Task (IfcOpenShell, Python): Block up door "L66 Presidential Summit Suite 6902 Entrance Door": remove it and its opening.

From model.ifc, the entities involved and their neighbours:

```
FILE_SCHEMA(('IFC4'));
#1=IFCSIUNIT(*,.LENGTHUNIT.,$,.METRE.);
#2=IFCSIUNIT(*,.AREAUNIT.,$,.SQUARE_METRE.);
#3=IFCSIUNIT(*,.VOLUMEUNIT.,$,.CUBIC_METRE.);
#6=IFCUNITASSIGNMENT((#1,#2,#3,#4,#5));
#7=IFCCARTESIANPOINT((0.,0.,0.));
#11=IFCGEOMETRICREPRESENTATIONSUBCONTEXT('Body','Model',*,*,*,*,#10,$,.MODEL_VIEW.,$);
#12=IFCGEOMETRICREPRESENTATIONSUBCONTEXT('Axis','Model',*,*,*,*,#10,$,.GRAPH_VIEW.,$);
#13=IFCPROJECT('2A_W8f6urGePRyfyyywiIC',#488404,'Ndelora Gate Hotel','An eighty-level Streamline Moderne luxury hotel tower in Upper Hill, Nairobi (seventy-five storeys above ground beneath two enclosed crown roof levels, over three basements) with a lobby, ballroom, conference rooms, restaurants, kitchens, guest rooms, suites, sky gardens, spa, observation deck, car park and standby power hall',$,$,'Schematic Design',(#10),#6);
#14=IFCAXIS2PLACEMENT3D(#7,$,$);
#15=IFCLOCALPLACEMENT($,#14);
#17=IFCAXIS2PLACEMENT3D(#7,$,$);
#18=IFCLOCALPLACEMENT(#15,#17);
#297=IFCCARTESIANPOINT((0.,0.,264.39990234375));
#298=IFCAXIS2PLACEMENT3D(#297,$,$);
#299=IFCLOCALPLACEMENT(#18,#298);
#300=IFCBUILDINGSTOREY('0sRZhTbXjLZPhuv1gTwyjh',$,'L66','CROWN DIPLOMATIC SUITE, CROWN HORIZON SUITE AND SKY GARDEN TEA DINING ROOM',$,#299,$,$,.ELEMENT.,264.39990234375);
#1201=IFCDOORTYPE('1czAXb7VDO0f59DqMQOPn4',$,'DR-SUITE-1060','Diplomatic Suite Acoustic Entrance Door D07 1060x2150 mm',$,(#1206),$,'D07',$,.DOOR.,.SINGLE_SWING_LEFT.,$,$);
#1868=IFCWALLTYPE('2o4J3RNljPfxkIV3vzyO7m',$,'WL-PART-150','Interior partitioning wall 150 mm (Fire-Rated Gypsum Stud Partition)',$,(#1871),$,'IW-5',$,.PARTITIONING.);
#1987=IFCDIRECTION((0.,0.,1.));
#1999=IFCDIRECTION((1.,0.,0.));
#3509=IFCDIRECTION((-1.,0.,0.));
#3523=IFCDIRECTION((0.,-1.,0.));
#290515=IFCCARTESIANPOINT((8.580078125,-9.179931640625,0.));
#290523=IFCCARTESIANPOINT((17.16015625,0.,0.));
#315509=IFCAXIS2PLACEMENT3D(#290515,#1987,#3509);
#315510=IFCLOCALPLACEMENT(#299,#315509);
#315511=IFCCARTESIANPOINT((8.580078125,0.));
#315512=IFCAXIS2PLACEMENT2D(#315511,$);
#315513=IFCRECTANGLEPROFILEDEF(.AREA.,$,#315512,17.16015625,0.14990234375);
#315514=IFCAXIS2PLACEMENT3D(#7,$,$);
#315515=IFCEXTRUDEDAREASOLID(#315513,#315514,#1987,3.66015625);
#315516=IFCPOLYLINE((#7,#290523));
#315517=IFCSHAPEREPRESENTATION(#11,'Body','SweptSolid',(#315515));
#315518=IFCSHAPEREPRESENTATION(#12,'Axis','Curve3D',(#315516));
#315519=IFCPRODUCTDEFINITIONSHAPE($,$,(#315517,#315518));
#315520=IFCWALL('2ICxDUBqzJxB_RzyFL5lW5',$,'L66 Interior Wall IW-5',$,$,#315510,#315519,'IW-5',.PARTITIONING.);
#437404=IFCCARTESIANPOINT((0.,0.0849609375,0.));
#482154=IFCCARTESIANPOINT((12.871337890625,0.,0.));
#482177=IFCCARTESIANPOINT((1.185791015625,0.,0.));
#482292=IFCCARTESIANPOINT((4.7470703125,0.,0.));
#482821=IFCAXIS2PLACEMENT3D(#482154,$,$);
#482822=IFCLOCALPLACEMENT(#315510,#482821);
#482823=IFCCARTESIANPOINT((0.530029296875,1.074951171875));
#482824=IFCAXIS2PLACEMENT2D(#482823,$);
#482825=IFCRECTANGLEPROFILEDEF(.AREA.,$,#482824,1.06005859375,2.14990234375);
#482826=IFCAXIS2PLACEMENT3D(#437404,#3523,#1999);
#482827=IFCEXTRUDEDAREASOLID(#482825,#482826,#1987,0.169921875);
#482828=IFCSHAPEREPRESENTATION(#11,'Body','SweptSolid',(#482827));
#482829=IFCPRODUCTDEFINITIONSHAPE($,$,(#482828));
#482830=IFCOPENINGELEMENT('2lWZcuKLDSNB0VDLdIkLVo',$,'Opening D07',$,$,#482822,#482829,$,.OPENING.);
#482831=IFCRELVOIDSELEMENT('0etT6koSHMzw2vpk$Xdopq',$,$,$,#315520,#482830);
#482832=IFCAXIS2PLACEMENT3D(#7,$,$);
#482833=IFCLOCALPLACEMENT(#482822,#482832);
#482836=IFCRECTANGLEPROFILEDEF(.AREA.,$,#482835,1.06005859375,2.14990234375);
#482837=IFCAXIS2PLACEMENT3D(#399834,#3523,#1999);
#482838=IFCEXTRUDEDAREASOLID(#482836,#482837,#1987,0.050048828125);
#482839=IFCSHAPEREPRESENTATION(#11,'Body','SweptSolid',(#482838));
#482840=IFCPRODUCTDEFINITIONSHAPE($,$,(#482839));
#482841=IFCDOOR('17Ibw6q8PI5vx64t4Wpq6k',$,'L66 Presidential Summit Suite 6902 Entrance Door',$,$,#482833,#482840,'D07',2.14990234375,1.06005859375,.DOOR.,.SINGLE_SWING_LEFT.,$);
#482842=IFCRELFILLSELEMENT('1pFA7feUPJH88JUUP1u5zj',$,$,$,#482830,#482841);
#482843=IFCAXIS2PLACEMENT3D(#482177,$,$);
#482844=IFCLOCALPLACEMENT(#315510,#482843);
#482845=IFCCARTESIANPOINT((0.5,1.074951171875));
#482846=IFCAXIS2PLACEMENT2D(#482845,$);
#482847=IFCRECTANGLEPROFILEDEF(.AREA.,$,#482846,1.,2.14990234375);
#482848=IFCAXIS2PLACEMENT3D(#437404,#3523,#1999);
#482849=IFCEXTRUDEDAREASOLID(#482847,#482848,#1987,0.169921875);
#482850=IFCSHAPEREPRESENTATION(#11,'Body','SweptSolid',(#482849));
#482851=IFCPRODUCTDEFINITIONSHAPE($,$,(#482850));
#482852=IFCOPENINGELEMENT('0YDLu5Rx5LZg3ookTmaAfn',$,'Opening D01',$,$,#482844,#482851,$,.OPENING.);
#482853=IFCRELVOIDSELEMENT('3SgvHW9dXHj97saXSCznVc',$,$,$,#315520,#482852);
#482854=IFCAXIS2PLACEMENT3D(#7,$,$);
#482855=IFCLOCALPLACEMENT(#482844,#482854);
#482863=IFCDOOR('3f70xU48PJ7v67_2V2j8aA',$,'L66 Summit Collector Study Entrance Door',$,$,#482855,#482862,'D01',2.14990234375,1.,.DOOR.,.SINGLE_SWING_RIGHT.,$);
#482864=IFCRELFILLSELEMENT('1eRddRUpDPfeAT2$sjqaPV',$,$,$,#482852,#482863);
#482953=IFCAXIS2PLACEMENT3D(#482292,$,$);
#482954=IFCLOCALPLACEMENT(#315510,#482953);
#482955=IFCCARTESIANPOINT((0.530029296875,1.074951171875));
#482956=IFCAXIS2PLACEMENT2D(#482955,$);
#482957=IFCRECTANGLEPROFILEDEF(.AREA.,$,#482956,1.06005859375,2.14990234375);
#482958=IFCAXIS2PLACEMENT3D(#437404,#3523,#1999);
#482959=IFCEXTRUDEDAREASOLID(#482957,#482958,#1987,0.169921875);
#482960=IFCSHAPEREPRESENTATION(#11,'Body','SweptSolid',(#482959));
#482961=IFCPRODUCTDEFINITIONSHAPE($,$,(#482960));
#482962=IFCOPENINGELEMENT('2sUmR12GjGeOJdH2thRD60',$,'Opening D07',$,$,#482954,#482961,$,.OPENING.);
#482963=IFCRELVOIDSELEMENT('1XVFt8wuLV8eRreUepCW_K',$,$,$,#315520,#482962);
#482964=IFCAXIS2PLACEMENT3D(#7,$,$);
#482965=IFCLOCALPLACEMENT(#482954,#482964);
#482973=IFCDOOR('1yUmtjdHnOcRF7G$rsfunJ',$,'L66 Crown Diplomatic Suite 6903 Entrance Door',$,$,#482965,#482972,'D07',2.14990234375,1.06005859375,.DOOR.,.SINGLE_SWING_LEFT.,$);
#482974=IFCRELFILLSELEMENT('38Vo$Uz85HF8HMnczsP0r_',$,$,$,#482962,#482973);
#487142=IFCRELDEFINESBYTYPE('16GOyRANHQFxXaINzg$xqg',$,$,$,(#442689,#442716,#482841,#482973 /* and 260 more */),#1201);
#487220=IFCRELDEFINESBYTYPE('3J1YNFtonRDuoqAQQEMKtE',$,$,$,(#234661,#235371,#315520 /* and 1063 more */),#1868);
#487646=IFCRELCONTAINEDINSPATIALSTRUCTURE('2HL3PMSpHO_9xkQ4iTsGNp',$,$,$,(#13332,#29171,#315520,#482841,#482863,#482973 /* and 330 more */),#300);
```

```python
import ifcopenshell
import ifcopenshell.api.feature
import ifcopenshell.api.root
import ifcopenshell.geom
import ifcopenshell.util.shape

model = ifcopenshell.open("model.ifc")
settings = ifcopenshell.geom.settings()


def volume(element):
    """Net volume in cubic metres, openings subtracted."""
    shape = ifcopenshell.geom.create_shape(settings, element)
    return ifcopenshell.util.shape.get_volume(shape.geometry)


door = model.by_guid("17Ibw6q8PI5vx64t4Wpq6k")
opening = door.FillsVoids[0].RelatingOpeningElement
wall = opening.VoidsElements[0].RelatingBuildingElement
before = volume(wall)

ifcopenshell.api.root.remove_product(model, product=door)
ifcopenshell.api.feature.remove_feature(model, feature=opening)

after = volume(wall)

print(f"wall volume {before:.3f} -> {after:.3f} m3")

model.write("model-out.ifc")
```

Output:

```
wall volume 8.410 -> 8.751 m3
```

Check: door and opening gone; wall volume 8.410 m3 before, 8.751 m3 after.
